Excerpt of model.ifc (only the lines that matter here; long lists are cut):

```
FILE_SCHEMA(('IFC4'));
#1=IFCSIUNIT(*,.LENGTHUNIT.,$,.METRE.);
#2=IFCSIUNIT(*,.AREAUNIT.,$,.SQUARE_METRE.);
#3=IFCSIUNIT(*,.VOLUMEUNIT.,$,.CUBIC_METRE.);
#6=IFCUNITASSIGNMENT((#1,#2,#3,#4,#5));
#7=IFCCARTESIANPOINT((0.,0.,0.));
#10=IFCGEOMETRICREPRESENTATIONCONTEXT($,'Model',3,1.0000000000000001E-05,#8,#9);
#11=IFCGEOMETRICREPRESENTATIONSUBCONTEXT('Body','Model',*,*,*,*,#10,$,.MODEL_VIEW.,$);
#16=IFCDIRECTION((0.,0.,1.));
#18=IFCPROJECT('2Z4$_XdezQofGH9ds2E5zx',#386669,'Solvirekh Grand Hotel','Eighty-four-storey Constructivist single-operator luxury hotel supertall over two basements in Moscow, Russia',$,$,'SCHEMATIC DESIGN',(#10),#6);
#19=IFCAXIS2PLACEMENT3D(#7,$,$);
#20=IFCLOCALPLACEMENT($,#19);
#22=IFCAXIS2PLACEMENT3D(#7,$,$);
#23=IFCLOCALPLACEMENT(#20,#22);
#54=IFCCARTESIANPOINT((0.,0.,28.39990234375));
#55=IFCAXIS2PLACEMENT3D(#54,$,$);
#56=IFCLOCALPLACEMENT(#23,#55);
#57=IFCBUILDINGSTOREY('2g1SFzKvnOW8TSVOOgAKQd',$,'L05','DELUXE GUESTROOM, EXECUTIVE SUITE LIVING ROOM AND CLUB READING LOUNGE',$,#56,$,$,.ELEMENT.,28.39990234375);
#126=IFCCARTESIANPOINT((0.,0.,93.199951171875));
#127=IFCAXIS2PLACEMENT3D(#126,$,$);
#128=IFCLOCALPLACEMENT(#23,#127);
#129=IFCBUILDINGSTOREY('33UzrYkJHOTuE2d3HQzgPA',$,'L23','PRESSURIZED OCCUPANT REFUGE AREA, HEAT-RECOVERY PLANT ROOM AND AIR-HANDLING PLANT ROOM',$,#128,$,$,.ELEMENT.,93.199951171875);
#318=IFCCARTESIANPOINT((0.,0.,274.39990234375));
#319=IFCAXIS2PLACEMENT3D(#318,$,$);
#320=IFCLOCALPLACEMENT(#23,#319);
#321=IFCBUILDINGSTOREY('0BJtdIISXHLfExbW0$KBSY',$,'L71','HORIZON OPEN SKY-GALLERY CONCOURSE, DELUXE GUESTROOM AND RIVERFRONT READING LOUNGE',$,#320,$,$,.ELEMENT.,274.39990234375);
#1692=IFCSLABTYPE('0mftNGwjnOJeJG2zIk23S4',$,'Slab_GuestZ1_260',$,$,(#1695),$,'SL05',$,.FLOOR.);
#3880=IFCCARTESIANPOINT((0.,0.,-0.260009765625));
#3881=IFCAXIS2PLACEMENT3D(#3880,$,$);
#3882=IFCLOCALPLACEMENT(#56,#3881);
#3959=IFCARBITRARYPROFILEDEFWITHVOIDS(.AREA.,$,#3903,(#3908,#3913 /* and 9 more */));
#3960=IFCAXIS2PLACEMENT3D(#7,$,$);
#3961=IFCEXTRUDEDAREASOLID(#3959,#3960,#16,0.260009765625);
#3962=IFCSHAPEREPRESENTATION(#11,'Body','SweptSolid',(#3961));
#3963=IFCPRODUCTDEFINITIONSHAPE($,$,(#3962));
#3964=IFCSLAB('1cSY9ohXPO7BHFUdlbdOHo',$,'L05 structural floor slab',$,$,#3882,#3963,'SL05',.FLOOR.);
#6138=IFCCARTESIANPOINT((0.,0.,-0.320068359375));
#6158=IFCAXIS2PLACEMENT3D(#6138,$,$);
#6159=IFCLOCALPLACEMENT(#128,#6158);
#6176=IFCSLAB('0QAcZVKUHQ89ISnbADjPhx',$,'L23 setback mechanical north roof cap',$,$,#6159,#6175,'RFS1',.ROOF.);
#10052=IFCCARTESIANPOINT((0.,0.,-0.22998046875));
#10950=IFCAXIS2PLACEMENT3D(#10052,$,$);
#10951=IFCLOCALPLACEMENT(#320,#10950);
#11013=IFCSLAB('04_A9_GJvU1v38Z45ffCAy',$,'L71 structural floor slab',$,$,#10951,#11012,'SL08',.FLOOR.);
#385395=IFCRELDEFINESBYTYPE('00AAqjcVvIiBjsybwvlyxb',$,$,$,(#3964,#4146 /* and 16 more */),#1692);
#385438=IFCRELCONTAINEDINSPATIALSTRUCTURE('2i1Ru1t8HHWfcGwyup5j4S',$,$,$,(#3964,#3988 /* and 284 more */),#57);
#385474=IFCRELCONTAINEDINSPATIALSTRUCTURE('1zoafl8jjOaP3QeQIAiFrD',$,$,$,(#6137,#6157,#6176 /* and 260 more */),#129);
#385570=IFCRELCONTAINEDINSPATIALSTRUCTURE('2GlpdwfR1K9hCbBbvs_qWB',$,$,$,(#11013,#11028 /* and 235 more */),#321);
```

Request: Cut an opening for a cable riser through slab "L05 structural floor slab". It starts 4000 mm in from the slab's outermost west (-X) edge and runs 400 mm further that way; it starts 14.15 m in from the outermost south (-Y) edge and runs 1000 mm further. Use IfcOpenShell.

```python
import numpy as np
import ifcopenshell
import ifcopenshell.api.feature
import ifcopenshell.api.geometry
import ifcopenshell.api.root
import ifcopenshell.geom
import ifcopenshell.util.placement
import ifcopenshell.util.representation
import ifcopenshell.util.shape
import ifcopenshell.util.unit

model = ifcopenshell.open("model.ifc")
unit_scale = ifcopenshell.util.unit.calculate_unit_scale(model)
settings = ifcopenshell.geom.settings()


def volume(element):
    """Net volume in cubic metres, openings subtracted."""
    shape = ifcopenshell.geom.create_shape(settings, element)
    return ifcopenshell.util.shape.get_volume(shape.geometry)


slab = model.by_guid("1cSY9ohXPO7BHFUdlbdOHo")
before = volume(slab)

# Extent in the slab's own axes, in metres. The edges named are its -X and -Y sides.
slab_shape = ifcopenshell.geom.create_shape(settings, slab)
vertices = ifcopenshell.util.shape.get_vertices(slab_shape.geometry)
x_min, y_min, bottom = vertices.min(axis=0)
top = vertices[:, 2].max()

opening = ifcopenshell.api.root.create_entity(model, ifc_class="IfcOpeningElement", name="Cable riser opening", predefined_type="OPENING")
context = ifcopenshell.util.representation.get_context(model, "Model", "Body", "MODEL_VIEW")
width, depth = 0.4, 1
outline = [(0.0, 0.0), (width, 0.0), (width, depth), (0.0, depth), (0.0, 0.0)]
# Overshoot both faces by 50 mm so the cut is clean.
shape = ifcopenshell.api.geometry.add_slab_representation(
    model, context=context, depth=top - bottom + 0.1, polyline=outline
)
ifcopenshell.api.geometry.assign_representation(model, product=opening, representation=shape)

matrix = ifcopenshell.util.placement.get_local_placement(slab.ObjectPlacement)
matrix[:, 3] = matrix @ np.append(np.array([x_min + 4, y_min + 14.15, bottom - 0.05]) / unit_scale, 1.0)
ifcopenshell.api.geometry.edit_object_placement(model, product=opening, matrix=matrix, is_si=False)
ifcopenshell.api.feature.add_feature(model, feature=opening, element=slab)

after = volume(slab)

print(f"slab volume {before:.3f} -> {after:.3f} m3")

model.write("model_rev.ifc")
```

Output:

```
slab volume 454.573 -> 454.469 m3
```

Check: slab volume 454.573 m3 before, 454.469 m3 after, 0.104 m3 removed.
